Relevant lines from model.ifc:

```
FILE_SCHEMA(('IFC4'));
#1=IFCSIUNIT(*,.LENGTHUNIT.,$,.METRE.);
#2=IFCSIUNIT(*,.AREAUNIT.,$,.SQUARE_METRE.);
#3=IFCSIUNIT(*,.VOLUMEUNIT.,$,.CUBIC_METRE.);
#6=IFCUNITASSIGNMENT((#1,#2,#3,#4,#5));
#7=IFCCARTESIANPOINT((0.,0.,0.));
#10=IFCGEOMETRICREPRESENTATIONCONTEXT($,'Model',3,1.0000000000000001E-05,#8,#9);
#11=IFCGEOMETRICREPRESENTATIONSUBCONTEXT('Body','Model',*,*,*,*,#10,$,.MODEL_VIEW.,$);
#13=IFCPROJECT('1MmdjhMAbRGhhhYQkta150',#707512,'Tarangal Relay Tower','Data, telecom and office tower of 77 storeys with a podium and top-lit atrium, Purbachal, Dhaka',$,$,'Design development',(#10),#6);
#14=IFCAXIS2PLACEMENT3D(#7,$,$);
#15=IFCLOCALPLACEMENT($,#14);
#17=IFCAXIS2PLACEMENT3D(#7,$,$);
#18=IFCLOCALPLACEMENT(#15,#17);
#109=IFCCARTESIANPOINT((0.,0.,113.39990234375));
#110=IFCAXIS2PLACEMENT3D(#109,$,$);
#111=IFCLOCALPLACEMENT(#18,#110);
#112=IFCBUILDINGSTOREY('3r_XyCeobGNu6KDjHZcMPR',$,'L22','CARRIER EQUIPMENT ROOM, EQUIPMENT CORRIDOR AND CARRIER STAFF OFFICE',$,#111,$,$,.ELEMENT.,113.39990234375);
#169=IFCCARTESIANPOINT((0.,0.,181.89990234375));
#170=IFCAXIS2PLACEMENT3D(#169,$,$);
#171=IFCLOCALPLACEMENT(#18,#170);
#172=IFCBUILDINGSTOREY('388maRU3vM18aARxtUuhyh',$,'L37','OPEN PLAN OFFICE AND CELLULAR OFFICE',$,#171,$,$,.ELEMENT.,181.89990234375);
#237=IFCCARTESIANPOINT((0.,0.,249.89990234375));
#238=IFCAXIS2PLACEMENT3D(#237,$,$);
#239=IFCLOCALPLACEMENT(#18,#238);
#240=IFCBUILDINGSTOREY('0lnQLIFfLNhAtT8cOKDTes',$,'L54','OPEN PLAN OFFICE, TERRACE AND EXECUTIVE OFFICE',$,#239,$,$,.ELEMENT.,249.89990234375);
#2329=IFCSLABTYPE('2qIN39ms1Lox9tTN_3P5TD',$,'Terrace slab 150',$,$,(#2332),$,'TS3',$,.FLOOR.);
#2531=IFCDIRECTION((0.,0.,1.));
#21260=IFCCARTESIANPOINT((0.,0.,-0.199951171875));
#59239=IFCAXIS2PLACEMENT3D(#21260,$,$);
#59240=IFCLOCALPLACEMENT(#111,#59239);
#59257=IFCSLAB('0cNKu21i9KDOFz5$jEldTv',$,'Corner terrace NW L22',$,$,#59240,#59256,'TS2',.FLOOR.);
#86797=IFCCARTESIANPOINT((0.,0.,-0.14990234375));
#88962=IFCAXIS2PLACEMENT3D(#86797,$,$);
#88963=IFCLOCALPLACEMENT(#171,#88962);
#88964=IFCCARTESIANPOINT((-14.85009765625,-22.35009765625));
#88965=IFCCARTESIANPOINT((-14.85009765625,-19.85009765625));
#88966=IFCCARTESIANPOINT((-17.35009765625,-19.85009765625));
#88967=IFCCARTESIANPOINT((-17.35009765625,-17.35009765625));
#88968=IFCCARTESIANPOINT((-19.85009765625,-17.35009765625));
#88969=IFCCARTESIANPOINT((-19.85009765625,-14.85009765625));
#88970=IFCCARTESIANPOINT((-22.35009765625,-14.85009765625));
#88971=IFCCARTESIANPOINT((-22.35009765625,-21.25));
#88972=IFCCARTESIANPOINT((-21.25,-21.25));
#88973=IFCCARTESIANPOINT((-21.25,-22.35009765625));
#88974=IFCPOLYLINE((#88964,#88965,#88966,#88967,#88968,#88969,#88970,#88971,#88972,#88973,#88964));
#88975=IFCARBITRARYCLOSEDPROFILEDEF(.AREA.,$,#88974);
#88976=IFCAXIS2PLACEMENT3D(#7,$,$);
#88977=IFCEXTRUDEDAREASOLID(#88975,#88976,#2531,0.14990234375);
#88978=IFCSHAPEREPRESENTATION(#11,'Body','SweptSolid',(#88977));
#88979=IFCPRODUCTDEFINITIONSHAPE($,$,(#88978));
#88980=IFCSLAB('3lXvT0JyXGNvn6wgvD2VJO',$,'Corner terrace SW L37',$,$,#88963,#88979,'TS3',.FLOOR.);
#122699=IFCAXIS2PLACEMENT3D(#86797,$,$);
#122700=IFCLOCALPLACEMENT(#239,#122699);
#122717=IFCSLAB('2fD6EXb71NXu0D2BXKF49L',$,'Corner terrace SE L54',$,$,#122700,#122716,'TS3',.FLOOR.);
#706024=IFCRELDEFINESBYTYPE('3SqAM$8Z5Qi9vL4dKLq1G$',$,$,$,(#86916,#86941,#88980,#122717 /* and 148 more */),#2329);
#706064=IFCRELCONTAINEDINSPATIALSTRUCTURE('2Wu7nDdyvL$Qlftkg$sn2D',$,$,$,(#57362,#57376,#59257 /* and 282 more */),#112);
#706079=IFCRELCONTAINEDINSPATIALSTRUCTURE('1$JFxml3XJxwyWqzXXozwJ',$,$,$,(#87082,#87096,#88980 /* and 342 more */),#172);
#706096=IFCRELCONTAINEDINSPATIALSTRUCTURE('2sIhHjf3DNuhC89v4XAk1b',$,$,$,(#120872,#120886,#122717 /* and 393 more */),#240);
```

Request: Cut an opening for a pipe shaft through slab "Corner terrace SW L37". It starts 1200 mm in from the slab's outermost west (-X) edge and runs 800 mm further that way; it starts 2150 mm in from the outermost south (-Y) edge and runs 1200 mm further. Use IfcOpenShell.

```python
import numpy as np
import ifcopenshell
import ifcopenshell.api.feature
import ifcopenshell.api.geometry
import ifcopenshell.api.root
import ifcopenshell.geom
import ifcopenshell.util.placement
import ifcopenshell.util.representation
import ifcopenshell.util.shape
import ifcopenshell.util.unit

model = ifcopenshell.open("model.ifc")
unit_scale = ifcopenshell.util.unit.calculate_unit_scale(model)
settings = ifcopenshell.geom.settings()


def volume(element):
    """Net volume in cubic metres, openings subtracted."""
    shape = ifcopenshell.geom.create_shape(settings, element)
    return ifcopenshell.util.shape.get_volume(shape.geometry)


slab = model.by_guid("3lXvT0JyXGNvn6wgvD2VJO")
before = volume(slab)

# Extent in the slab's own axes, in metres. The edges named are its -X and -Y sides.
slab_shape = ifcopenshell.geom.create_shape(settings, slab)
vertices = ifcopenshell.util.shape.get_vertices(slab_shape.geometry)
x_min, y_min, bottom = vertices.min(axis=0)
top = vertices[:, 2].max()

opening = ifcopenshell.api.root.create_entity(model, ifc_class="IfcOpeningElement", name="Pipe shaft opening", predefined_type="OPENING")
context = ifcopenshell.util.representation.get_context(model, "Model", "Body", "MODEL_VIEW")
width, depth = 0.8, 1.2
outline = [(0.0, 0.0), (width, 0.0), (width, depth), (0.0, depth), (0.0, 0.0)]
# Overshoot both faces by 50 mm so the cut is clean.
shape = ifcopenshell.api.geometry.add_slab_representation(
    model, context=context, depth=top - bottom + 0.1, polyline=outline
)
ifcopenshell.api.geometry.assign_representation(model, product=opening, representation=shape)

matrix = ifcopenshell.util.placement.get_local_placement(slab.ObjectPlacement)
matrix[:, 3] = matrix @ np.append(np.array([x_min + 1.2, y_min + 2.15, bottom - 0.05]) / unit_scale, 1.0)
ifcopenshell.api.geometry.edit_object_placement(model, product=opening, matrix=matrix, is_si=False)
ifcopenshell.api.feature.add_feature(model, feature=opening, element=slab)

after = volume(slab)

print(f"slab volume {before:.3f} -> {after:.3f} m3")

model.write("model_edited.ifc")
```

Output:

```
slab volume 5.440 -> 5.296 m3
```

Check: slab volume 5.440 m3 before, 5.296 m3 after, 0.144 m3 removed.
